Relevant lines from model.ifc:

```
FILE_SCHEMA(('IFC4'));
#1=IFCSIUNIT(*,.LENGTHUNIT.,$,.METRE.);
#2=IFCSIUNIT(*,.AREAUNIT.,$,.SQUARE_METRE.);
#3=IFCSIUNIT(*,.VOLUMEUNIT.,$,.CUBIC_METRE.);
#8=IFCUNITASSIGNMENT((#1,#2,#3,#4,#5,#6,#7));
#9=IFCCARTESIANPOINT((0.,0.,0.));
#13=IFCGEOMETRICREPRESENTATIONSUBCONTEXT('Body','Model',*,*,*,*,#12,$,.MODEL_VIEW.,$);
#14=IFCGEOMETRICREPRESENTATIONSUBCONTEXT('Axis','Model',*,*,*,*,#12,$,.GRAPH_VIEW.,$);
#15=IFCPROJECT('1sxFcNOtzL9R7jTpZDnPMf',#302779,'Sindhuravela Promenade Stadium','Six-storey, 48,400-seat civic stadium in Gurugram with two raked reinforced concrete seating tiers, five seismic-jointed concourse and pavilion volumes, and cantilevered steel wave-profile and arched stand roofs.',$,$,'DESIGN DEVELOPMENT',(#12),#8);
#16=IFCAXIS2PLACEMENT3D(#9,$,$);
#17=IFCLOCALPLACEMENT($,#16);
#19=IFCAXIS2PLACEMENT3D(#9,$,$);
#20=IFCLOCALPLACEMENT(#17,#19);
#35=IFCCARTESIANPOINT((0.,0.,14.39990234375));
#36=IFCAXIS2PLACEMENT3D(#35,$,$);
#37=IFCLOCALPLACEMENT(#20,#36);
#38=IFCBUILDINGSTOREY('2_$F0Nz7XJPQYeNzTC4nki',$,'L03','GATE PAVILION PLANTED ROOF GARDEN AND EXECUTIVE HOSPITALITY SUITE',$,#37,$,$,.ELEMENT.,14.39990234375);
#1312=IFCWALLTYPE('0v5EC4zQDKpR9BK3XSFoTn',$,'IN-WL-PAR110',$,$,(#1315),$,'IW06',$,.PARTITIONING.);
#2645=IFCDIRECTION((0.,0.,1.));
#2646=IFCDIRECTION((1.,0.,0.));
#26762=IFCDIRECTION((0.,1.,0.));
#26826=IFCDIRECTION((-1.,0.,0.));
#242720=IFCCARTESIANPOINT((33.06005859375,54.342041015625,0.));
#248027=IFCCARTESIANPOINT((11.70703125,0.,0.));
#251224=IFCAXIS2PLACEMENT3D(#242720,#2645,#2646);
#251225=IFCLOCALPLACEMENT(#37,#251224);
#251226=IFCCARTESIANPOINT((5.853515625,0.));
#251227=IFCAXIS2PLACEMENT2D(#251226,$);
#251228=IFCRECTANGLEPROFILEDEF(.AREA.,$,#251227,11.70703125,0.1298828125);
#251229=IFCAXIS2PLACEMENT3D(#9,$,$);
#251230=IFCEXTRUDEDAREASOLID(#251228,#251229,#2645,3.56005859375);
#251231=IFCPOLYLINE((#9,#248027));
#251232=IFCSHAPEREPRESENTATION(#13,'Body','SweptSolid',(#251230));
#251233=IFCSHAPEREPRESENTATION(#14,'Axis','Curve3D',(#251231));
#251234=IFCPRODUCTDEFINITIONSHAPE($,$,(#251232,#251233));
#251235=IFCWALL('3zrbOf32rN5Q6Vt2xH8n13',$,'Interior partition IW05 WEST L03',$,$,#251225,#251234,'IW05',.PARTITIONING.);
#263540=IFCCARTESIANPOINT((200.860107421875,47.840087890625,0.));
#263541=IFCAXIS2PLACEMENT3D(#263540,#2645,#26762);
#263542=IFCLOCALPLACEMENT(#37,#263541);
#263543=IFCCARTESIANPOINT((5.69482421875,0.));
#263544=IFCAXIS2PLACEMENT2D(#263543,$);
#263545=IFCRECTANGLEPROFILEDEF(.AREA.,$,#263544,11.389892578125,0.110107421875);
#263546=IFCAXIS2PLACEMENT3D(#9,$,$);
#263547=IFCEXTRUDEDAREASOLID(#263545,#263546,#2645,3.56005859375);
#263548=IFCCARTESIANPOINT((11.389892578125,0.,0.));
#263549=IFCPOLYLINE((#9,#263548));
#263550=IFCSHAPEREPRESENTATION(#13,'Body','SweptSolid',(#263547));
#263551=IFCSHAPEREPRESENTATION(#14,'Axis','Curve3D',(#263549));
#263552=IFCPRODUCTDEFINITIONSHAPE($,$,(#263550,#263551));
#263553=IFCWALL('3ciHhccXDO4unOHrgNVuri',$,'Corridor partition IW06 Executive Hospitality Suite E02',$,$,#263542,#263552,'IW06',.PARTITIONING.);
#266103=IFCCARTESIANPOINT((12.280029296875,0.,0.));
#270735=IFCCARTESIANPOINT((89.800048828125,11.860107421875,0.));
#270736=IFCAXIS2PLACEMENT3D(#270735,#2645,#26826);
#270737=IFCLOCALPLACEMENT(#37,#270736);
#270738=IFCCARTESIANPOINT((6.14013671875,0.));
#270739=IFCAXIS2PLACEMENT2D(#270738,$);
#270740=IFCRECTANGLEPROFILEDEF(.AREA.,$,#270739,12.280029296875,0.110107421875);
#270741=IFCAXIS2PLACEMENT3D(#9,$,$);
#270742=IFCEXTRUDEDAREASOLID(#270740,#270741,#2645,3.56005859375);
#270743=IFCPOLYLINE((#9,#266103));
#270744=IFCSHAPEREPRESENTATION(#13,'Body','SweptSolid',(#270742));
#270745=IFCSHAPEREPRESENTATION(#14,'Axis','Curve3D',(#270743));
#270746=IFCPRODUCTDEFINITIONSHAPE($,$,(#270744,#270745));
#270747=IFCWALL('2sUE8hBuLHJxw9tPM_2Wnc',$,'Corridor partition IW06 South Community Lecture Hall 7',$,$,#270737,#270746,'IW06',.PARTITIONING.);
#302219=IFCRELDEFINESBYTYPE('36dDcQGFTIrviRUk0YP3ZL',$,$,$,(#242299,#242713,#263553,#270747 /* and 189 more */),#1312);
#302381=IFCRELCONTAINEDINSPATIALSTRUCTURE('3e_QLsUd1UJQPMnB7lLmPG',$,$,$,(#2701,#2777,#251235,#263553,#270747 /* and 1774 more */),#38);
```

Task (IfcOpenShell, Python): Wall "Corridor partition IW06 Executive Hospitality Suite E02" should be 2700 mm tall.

```python
import ifcopenshell
import ifcopenshell.geom
import ifcopenshell.util.representation
import ifcopenshell.util.shape
import ifcopenshell.util.unit

model = ifcopenshell.open("model.ifc")
unit_scale = ifcopenshell.util.unit.calculate_unit_scale(model)
settings = ifcopenshell.geom.settings()


def volume(element):
    """Net volume in cubic metres, openings subtracted."""
    shape = ifcopenshell.geom.create_shape(settings, element)
    return ifcopenshell.util.shape.get_volume(shape.geometry)


wall = model.by_guid("3ciHhccXDO4unOHrgNVuri")
before = volume(wall)

body = ifcopenshell.util.representation.get_representation(wall, "Model", "Body")
solid = body.Items[0]
old_height = solid.Depth
solid.Depth = 2.7 / unit_scale
after = volume(wall)

print(f"height {old_height:g} -> {solid.Depth:g}, volume {before:.3f} -> {after:.3f} m3")

model.write("model_updated.ifc")
```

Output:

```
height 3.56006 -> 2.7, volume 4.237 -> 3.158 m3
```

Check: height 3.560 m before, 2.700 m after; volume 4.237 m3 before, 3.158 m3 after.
